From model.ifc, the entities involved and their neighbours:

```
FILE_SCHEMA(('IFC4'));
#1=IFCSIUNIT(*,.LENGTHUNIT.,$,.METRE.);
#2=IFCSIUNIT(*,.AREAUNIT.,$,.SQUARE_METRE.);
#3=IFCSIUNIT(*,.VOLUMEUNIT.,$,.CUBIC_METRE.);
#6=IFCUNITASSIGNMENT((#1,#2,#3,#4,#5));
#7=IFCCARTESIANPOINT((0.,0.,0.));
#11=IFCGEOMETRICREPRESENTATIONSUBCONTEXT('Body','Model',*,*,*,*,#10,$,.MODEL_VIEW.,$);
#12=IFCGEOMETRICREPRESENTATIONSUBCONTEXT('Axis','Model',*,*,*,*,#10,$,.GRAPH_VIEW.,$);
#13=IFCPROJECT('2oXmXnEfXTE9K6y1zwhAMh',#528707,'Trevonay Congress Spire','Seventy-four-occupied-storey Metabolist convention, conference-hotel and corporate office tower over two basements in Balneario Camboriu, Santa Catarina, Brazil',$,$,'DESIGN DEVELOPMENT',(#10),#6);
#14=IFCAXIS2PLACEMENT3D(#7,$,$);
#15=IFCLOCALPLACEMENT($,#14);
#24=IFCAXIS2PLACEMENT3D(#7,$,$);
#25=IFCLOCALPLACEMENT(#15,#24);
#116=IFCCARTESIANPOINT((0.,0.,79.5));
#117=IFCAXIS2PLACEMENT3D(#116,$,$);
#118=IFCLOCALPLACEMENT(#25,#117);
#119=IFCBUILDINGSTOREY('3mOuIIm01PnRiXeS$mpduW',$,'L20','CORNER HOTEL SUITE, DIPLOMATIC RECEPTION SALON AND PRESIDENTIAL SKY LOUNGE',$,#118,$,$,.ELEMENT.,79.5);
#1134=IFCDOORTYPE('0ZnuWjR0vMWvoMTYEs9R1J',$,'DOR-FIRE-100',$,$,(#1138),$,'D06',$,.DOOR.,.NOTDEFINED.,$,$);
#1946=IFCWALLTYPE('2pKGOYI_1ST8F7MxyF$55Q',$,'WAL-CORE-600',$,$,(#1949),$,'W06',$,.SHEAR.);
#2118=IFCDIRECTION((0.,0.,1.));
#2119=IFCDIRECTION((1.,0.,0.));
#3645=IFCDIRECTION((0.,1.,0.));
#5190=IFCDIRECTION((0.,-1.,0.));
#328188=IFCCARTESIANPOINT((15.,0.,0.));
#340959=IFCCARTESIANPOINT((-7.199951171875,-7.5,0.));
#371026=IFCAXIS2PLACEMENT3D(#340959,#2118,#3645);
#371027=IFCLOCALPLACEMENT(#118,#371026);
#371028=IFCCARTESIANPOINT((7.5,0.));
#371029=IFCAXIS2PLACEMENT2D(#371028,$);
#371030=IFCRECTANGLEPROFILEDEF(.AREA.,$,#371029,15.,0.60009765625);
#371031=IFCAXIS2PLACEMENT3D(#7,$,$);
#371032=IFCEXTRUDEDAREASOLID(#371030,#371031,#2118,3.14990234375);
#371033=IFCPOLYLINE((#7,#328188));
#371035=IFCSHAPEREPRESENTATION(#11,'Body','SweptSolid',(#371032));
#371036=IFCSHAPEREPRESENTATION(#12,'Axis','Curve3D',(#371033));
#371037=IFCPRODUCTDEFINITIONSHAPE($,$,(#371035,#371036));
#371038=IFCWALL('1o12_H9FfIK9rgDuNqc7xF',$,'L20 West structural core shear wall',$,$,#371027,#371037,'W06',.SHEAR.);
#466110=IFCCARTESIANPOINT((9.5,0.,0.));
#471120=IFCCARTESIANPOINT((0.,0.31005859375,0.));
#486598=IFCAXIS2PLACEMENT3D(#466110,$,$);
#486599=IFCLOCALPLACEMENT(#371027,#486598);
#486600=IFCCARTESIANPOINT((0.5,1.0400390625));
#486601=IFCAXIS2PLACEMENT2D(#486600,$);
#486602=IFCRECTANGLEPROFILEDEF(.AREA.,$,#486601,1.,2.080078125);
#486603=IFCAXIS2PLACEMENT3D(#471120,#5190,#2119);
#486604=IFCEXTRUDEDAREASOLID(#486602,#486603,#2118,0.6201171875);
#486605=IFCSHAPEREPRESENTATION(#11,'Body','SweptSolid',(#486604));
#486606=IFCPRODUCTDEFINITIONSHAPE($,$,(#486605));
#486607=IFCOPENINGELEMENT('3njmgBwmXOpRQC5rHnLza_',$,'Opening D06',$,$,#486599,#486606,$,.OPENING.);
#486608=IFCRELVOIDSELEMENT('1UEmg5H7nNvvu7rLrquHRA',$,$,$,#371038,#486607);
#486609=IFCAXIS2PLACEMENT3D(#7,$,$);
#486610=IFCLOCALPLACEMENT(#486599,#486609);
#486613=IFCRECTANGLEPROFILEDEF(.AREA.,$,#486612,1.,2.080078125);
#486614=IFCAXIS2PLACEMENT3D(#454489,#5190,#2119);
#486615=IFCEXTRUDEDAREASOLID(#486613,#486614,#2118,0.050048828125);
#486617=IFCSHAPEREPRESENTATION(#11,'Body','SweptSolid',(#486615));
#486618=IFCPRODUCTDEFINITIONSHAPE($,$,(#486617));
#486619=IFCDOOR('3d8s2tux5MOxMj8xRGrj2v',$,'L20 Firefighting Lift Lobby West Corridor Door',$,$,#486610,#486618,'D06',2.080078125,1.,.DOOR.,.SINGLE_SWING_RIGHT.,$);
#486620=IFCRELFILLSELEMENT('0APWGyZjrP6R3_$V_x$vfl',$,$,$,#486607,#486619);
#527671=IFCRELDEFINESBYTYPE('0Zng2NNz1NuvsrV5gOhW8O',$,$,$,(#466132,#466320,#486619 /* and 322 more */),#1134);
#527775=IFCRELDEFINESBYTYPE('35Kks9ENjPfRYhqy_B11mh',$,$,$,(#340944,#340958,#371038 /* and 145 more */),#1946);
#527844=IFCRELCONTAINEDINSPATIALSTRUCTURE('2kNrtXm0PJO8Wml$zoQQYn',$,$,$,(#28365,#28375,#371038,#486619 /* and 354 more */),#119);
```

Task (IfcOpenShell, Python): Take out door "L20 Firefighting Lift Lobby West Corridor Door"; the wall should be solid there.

```python
import ifcopenshell
import ifcopenshell.api.feature
import ifcopenshell.api.root
import ifcopenshell.geom
import ifcopenshell.util.shape

model = ifcopenshell.open("model.ifc")
settings = ifcopenshell.geom.settings()


def volume(element):
    """Net volume in cubic metres, openings subtracted."""
    shape = ifcopenshell.geom.create_shape(settings, element)
    return ifcopenshell.util.shape.get_volume(shape.geometry)


door = model.by_guid("3d8s2tux5MOxMj8xRGrj2v")
opening = door.FillsVoids[0].RelatingOpeningElement
wall = opening.VoidsElements[0].RelatingBuildingElement
before = volume(wall)

ifcopenshell.api.root.remove_product(model, product=door)
ifcopenshell.api.feature.remove_feature(model, feature=opening)

after = volume(wall)

print(f"wall volume {before:.3f} -> {after:.3f} m3")

model.write("model_v2.ifc")
```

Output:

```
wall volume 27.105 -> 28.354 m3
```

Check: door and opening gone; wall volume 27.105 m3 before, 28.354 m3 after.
